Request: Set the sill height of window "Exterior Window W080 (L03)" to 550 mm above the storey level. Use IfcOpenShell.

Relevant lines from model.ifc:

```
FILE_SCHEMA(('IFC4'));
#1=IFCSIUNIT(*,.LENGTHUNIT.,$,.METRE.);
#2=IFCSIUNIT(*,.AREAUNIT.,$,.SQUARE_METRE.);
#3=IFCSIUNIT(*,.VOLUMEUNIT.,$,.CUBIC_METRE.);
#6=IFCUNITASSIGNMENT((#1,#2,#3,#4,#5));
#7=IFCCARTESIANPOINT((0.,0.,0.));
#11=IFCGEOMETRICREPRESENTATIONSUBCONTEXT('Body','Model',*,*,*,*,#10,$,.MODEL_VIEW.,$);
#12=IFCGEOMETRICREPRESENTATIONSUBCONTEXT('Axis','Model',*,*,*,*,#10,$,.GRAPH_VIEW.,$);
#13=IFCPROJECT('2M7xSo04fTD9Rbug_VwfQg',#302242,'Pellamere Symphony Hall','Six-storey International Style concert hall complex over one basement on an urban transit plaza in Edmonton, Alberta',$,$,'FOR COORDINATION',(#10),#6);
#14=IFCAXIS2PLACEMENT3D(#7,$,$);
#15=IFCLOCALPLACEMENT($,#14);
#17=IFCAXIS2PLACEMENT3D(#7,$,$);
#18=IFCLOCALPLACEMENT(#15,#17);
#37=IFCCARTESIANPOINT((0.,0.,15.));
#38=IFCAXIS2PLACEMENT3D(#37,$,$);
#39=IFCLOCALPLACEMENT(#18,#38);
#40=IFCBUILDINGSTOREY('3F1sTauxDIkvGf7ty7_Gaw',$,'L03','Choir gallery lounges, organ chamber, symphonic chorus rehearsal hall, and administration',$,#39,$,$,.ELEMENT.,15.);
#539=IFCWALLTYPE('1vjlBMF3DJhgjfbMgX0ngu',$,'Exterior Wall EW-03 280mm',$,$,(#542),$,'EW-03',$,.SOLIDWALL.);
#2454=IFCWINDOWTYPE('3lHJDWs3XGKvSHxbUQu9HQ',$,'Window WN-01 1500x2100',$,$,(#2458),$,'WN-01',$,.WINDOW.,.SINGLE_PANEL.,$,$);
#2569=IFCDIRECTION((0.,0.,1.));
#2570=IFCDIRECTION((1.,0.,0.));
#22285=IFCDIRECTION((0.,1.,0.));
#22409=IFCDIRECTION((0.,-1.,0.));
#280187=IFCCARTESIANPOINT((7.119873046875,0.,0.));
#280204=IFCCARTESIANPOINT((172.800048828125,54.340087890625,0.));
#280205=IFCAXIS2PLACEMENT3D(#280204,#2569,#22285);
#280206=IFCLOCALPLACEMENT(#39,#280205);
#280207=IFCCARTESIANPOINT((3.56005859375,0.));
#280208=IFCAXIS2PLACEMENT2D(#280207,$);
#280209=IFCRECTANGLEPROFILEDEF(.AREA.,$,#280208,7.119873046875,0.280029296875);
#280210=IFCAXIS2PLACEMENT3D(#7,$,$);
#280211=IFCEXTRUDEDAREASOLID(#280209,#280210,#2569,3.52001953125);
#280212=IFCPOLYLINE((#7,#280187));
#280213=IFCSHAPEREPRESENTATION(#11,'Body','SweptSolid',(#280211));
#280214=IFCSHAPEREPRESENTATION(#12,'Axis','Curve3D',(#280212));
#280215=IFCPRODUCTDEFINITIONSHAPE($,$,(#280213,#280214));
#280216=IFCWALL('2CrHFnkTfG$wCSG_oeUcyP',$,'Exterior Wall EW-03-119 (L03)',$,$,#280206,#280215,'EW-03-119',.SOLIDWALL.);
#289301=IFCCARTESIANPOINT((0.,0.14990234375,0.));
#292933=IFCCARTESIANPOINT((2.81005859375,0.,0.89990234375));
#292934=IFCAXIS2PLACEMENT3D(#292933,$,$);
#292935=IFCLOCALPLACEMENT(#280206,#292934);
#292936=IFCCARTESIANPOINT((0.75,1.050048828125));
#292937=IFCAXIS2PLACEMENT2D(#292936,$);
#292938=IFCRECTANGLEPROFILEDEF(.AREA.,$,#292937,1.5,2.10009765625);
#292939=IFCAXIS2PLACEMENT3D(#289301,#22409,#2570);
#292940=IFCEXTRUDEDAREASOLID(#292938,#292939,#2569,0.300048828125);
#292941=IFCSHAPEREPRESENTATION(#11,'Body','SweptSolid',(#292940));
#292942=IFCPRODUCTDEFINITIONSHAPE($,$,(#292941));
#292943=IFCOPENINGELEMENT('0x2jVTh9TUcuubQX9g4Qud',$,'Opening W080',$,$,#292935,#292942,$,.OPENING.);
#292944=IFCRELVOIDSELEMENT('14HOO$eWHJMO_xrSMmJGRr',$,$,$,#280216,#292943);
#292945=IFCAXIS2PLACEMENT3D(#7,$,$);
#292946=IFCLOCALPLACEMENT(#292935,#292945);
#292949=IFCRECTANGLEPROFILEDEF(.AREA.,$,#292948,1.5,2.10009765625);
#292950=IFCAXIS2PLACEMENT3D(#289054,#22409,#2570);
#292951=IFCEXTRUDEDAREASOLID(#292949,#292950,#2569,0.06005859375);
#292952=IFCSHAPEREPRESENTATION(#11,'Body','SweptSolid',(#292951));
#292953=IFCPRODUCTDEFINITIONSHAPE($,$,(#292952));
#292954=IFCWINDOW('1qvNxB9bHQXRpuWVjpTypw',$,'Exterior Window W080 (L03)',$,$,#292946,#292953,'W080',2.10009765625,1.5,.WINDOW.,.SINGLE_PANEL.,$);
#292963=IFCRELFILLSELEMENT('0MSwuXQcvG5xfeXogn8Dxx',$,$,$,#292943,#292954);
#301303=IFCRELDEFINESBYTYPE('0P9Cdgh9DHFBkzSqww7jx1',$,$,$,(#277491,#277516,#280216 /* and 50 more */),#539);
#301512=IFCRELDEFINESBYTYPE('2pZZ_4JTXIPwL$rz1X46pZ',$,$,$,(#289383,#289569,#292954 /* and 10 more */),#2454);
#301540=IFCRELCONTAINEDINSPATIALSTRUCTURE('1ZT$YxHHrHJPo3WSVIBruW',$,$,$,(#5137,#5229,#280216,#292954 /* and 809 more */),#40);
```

```python
import numpy as np
import ifcopenshell
import ifcopenshell.api.geometry
import ifcopenshell.geom
import ifcopenshell.util.element
import ifcopenshell.util.placement
import ifcopenshell.util.shape
import ifcopenshell.util.unit

model = ifcopenshell.open("model.ifc")
unit_scale = ifcopenshell.util.unit.calculate_unit_scale(model)

window = model.by_id(292954)
opening = window.FillsVoids[0].RelatingOpeningElement
storey = ifcopenshell.util.element.get_container(window, ifc_class="IfcBuildingStorey")
level = ifcopenshell.util.placement.get_local_placement(storey.ObjectPlacement)[2, 3]

# The opening's origin need not be at the sill, so measure its lowest point.
shape = ifcopenshell.geom.create_shape(ifcopenshell.geom.settings(), opening)
bottom = ifcopenshell.util.shape.get_shape_bottom_elevation(shape, shape.geometry) / unit_scale
dz = level + 0.55 / unit_scale - bottom

shift = np.array([0.0, 0.0, dz])
# The window is placed relative to its opening, so it follows when the opening moves.
matrix = ifcopenshell.util.placement.get_local_placement(opening.ObjectPlacement)
matrix[:3, 3] += shift
ifcopenshell.api.geometry.edit_object_placement(
    model, product=opening, matrix=matrix, is_si=False, should_transform_children=True
)

print(f"moved by {dz * unit_scale:+.3f} m")

model.write("model-out.ifc")
```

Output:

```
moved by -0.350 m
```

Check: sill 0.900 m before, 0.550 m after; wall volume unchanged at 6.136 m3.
